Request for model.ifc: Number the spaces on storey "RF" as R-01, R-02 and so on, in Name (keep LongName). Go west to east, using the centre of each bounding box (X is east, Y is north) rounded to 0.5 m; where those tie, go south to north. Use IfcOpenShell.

First a look at what the model holds.

```python
import ifcopenshell
import ifcopenshell.util.element
import ifcopenshell.util.placement

model = ifcopenshell.open("model.ifc")
print(model.schema)
storey = next(s for s in model.by_type("IfcBuildingStorey") if s.Name == "RF")
spaces = [e for e in ifcopenshell.util.element.get_decomposition(storey) if e.is_a("IfcSpace")]
for e in sorted(spaces, key=lambda e: e.id()):
    origin = ifcopenshell.util.placement.get_local_placement(e.ObjectPlacement)[:3, 3]
    print(e.id(), e.Name, e.LongName, origin.round(2) + 0.0, sep=" | ")
```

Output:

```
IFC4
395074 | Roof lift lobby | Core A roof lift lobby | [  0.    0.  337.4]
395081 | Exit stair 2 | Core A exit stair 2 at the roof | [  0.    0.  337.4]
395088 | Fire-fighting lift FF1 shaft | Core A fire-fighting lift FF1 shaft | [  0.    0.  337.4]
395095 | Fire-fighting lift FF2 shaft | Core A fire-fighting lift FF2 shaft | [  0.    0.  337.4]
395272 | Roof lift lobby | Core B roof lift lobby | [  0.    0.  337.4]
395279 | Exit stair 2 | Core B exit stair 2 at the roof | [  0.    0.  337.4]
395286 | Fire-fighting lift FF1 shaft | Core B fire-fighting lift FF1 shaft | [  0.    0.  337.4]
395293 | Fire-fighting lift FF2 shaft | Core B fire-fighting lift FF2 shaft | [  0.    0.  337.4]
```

```python
import ifcopenshell
import ifcopenshell.geom
import ifcopenshell.util.element
import ifcopenshell.util.shape

model = ifcopenshell.open("model.ifc")
settings = ifcopenshell.geom.settings()
settings.set("use-world-coords", True)


def centre(element):
    shape = ifcopenshell.geom.create_shape(settings, element)
    return ifcopenshell.util.shape.get_bbox_centroid(shape.geometry)


storey = next(s for s in model.by_type("IfcBuildingStorey") if s.Name == "RF")
spaces = [e for e in ifcopenshell.util.element.get_decomposition(storey) if e.is_a("IfcSpace")]

# Insertion points can sit at a corner or the storey origin, so sort by the geometry (in metres).
centres = {e: centre(e) for e in spaces}
spaces.sort(key=lambda e: (round(centres[e][0] / 0.5), centres[e][1]))

for i, e in enumerate(spaces, start=1):
    number = f"R-{i:02d}"
    e.Name = number
    print(e.id(), number)

model.write("model_updated.ifc")
```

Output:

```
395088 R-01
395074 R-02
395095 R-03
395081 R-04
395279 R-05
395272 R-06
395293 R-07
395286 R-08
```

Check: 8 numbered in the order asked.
